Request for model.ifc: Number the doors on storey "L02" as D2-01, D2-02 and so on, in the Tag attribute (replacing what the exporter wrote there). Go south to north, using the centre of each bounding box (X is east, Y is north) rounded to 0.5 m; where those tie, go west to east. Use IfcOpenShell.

First a look at what the model holds.

```python
import ifcopenshell
import ifcopenshell.util.element
import ifcopenshell.util.placement

model = ifcopenshell.open("model.ifc")
print(model.schema)
storey = next(s for s in model.by_type("IfcBuildingStorey") if s.Name == "L02")
doors = [e for e in ifcopenshell.util.element.get_decomposition(storey) if e.is_a("IfcDoor")]
for e in sorted(doors, key=lambda e: e.id()):
    origin = ifcopenshell.util.placement.get_local_placement(e.ObjectPlacement)[:3, 3]
    print(e.id(), e.Tag, e.Name, origin.round(2) + 0.0, sep=" | ")
```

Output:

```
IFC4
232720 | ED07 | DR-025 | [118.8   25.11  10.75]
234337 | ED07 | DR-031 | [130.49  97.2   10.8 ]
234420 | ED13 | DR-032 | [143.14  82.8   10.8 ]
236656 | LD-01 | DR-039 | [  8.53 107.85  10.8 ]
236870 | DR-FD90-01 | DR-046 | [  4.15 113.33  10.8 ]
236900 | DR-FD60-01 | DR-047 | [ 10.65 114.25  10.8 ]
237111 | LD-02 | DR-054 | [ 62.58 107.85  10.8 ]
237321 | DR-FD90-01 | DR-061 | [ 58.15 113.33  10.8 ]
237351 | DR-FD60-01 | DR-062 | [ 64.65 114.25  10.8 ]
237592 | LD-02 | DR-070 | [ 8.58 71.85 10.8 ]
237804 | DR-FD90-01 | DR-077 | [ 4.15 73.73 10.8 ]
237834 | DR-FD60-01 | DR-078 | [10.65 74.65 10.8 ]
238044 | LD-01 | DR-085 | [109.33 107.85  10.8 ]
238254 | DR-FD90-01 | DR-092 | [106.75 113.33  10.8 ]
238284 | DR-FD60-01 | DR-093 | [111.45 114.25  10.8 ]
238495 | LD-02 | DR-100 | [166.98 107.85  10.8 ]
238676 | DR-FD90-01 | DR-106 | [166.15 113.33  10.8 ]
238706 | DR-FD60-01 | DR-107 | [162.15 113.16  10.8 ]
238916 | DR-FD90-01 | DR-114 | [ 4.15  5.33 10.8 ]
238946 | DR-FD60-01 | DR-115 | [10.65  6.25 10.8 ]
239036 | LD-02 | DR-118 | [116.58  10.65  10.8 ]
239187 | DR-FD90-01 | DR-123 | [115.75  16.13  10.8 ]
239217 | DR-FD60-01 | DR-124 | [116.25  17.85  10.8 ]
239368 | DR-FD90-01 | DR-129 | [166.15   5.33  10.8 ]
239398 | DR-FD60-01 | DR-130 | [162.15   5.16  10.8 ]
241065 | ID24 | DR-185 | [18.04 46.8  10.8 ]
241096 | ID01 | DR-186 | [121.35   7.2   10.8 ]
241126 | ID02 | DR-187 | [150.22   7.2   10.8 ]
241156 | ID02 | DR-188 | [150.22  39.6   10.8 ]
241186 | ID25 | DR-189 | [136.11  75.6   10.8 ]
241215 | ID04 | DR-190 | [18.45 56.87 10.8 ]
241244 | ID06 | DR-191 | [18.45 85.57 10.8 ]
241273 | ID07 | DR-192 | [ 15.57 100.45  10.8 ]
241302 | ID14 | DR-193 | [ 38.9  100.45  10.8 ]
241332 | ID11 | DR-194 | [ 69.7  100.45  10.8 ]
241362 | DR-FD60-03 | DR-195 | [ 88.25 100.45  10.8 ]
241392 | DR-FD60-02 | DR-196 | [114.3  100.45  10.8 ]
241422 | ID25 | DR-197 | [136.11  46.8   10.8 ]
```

```python
import ifcopenshell
import ifcopenshell.geom
import ifcopenshell.util.element
import ifcopenshell.util.shape

model = ifcopenshell.open("model.ifc")
settings = ifcopenshell.geom.settings()
settings.set("use-world-coords", True)


def centre(element):
    shape = ifcopenshell.geom.create_shape(settings, element)
    return ifcopenshell.util.shape.get_bbox_centroid(shape.geometry)


storey = next(s for s in model.by_type("IfcBuildingStorey") if s.Name == "L02")
doors = [e for e in ifcopenshell.util.element.get_decomposition(storey) if e.is_a("IfcDoor")]

# Insertion points can sit at a corner or the storey origin, so sort by the geometry (in metres).
centres = {e: centre(e) for e in doors}
doors.sort(key=lambda e: (round(centres[e][1] / 0.5), centres[e][0]))

for i, e in enumerate(doors, start=1):
    number = f"D2-{i:02d}"
    e.Tag = number
    print(e.id(), number)

model.write("model_updated.ifc")
```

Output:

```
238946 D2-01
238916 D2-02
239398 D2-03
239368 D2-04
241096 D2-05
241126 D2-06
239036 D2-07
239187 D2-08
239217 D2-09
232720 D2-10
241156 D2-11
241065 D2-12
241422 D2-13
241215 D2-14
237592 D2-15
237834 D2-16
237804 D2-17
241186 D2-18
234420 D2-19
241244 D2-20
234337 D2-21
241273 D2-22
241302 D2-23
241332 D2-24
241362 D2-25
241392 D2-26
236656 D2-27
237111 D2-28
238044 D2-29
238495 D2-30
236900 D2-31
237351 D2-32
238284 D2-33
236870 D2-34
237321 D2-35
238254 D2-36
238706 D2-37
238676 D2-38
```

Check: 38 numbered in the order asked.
